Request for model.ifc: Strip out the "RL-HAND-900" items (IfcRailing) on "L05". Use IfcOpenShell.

First a look at what the model holds.

```python
import ifcopenshell
import ifcopenshell.util.element

model = ifcopenshell.open("model.ifc")
print(model.schema)
storey = next(s for s in model.by_type("IfcBuildingStorey") if s.Name == "L05")
railings = [e for e in ifcopenshell.util.element.get_decomposition(storey) if e.is_a("IfcRailing")]
seen = {}
for e in railings:
    element_type = ifcopenshell.util.element.get_type(e)
    name = element_type.Name if element_type not in (None, e) else None
    seen[name] = seen.get(name, 0) + 1
for name, count in sorted(seen.items(), key=str):
    print(count, "x", name)
```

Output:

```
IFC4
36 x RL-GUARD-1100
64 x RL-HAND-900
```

```python
import ifcopenshell
import ifcopenshell.api.root
import ifcopenshell.util.element

model = ifcopenshell.open("model.ifc")

storey = next(s for s in model.by_type("IfcBuildingStorey") if s.Name == "L05")
railings = [e for e in ifcopenshell.util.element.get_decomposition(storey) if e.is_a("IfcRailing")]
targets = [e for e in railings if (t := ifcopenshell.util.element.get_type(e)) not in (None, e) and t.Name == "RL-HAND-900"]

for e in targets:
    ifcopenshell.api.root.remove_product(model, product=e)
print(len(targets), "removed")

model.write("model-out.ifc")
```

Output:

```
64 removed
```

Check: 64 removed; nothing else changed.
